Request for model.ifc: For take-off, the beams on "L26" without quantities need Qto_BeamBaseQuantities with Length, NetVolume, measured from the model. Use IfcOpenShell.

First a look at what the model holds.

```python
import ifcopenshell
import ifcopenshell.util.element
import ifcopenshell.util.unit

model = ifcopenshell.open("model.ifc")
print(model.schema)
for unit_type in ("LENGTHUNIT", "AREAUNIT", "VOLUMEUNIT"):
    print(unit_type, ifcopenshell.util.unit.calculate_unit_scale(model, unit_type))
storey = next(s for s in model.by_type("IfcBuildingStorey") if s.Name == "L26")
beams = [e for e in ifcopenshell.util.element.get_decomposition(storey) if e.is_a("IfcBeam")]
for e in sorted(beams, key=lambda e: e.id()):
    print(e.id(), e.is_a(), e.Name, list(ifcopenshell.util.element.get_psets(e, qtos_only=True)), sep=" | ")
```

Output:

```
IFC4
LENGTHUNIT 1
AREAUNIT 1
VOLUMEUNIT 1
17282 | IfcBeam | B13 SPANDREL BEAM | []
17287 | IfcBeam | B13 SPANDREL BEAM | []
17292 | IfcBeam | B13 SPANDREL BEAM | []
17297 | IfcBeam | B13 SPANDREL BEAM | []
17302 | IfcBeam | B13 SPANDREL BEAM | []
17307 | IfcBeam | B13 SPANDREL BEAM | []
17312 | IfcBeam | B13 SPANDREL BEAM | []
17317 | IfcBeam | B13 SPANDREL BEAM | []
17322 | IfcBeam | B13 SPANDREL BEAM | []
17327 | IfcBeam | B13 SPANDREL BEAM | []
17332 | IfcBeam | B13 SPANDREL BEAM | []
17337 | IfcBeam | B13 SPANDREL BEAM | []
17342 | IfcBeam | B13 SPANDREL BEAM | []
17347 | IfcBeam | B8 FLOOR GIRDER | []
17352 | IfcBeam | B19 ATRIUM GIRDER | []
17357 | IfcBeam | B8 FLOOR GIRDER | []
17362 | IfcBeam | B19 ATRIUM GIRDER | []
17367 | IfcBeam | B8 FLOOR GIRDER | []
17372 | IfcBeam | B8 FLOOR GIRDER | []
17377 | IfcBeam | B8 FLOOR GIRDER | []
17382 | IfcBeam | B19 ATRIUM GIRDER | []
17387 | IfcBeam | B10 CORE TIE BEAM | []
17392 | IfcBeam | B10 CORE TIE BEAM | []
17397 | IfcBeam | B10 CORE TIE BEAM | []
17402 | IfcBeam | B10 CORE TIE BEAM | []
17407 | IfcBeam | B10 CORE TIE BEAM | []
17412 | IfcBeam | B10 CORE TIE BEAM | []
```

```python
import ifcopenshell
import ifcopenshell.api.pset
import ifcopenshell.geom
import ifcopenshell.util.element
import ifcopenshell.util.shape
import ifcopenshell.util.unit

model = ifcopenshell.open("model.ifc")
unit_scale = ifcopenshell.util.unit.calculate_unit_scale(model)
volume_scale = ifcopenshell.util.unit.calculate_unit_scale(model, "VOLUMEUNIT")
settings = ifcopenshell.geom.settings()

storey = next(s for s in model.by_type("IfcBuildingStorey") if s.Name == "L26")
beams = [e for e in ifcopenshell.util.element.get_decomposition(storey) if e.is_a("IfcBeam")]

for e in sorted(beams, key=lambda e: e.id()):
    if ifcopenshell.util.element.get_psets(e, qtos_only=True, should_inherit=False):
        continue
    # Geometry comes back in metres, in the element's own axes.
    shape = ifcopenshell.geom.create_shape(settings, e)
    values = {
        "Length": ifcopenshell.util.shape.get_max_xyz(shape.geometry) / unit_scale,
        "NetVolume": ifcopenshell.util.shape.get_volume(shape.geometry) / volume_scale,
    }
    qto = ifcopenshell.api.pset.add_qto(model, product=e, name="Qto_BeamBaseQuantities")
    ifcopenshell.api.pset.edit_qto(model, qto=qto, properties=values)
    print(e.id(), {k: round(v, 3) for k, v in values.items()})

model.write("model_rev.ifc")
```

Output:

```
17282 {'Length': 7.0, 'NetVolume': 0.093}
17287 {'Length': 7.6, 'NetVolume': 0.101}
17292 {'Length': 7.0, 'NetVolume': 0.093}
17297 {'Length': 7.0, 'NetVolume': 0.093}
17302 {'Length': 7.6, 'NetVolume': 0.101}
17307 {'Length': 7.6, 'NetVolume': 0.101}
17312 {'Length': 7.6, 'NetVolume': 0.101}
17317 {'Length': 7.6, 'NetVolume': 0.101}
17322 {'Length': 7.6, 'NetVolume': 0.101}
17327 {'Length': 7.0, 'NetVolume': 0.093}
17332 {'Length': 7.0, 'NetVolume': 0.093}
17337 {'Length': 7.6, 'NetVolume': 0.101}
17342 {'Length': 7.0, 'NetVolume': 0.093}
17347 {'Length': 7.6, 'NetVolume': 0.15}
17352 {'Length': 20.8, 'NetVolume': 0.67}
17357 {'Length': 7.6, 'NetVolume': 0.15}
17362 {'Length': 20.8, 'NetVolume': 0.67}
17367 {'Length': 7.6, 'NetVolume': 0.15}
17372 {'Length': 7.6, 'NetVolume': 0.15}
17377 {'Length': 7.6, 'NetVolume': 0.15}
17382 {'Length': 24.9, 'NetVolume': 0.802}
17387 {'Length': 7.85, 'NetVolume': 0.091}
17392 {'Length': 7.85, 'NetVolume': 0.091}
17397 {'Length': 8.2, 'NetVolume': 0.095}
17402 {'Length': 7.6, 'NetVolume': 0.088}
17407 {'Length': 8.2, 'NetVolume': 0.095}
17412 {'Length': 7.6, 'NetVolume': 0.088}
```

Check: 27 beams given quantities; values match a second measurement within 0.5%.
